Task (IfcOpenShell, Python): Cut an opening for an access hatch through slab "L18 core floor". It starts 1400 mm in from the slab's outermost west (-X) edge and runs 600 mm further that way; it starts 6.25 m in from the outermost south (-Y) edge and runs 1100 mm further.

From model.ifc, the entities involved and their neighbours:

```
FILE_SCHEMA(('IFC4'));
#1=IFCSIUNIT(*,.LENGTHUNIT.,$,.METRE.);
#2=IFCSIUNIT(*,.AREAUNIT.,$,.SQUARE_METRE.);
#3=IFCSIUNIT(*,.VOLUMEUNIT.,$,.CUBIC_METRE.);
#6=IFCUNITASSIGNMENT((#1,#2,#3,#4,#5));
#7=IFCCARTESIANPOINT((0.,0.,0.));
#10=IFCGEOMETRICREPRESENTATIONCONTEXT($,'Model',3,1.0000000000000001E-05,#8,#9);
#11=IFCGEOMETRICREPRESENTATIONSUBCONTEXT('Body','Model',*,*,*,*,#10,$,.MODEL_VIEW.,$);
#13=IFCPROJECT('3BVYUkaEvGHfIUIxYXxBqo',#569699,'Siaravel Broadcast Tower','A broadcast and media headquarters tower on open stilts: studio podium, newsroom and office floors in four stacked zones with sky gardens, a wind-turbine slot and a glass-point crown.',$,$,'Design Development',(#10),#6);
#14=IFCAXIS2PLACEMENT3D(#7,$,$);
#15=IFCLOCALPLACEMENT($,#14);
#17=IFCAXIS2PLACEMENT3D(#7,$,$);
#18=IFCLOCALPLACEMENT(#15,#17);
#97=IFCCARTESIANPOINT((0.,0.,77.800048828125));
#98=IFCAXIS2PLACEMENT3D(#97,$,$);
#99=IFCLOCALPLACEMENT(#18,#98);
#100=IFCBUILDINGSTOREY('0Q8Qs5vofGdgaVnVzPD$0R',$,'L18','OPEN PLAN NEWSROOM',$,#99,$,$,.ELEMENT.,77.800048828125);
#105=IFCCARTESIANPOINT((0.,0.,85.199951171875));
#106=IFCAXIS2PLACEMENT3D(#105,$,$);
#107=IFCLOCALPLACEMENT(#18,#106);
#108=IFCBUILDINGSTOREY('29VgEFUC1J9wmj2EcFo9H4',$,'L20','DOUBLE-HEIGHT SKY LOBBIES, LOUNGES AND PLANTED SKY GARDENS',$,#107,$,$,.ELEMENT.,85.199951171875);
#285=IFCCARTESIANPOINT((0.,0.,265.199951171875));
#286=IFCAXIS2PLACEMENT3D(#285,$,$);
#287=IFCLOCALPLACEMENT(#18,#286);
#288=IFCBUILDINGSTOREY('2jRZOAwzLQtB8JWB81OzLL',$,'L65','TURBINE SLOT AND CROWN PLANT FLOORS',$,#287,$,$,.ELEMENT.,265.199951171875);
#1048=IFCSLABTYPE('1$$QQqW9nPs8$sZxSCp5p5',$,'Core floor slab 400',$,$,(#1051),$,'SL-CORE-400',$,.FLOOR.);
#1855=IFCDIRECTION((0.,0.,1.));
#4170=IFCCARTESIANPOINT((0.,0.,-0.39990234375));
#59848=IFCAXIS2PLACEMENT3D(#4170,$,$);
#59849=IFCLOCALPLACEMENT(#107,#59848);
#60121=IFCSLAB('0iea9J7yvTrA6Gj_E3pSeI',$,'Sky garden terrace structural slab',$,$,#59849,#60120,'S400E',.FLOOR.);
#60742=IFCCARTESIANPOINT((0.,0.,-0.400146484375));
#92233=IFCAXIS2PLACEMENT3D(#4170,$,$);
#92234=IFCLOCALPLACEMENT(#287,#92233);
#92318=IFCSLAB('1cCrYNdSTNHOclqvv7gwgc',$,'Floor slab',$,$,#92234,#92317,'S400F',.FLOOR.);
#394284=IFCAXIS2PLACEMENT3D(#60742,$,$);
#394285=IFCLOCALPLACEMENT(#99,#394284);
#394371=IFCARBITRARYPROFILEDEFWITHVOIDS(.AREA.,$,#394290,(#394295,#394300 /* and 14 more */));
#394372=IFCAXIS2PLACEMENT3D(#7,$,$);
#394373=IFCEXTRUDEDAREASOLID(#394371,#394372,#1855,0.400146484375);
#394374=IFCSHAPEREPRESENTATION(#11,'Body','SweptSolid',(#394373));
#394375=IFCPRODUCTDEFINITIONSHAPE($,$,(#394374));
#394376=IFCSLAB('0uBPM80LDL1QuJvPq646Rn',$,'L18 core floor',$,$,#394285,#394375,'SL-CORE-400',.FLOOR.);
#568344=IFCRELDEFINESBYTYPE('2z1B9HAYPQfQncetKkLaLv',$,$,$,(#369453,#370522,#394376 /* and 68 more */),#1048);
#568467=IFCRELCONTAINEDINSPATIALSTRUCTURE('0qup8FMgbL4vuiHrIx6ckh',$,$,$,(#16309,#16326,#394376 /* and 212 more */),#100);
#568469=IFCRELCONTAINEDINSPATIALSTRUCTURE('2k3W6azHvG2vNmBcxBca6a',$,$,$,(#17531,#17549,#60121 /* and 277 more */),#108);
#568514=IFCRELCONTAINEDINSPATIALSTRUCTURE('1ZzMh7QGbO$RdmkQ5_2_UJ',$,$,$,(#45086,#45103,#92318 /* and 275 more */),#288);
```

```python
import numpy as np
import ifcopenshell
import ifcopenshell.api.feature
import ifcopenshell.api.geometry
import ifcopenshell.api.root
import ifcopenshell.geom
import ifcopenshell.util.placement
import ifcopenshell.util.representation
import ifcopenshell.util.shape
import ifcopenshell.util.unit

model = ifcopenshell.open("model.ifc")
unit_scale = ifcopenshell.util.unit.calculate_unit_scale(model)
settings = ifcopenshell.geom.settings()


def volume(element):
    """Net volume in cubic metres, openings subtracted."""
    shape = ifcopenshell.geom.create_shape(settings, element)
    return ifcopenshell.util.shape.get_volume(shape.geometry)


slab = model.by_guid("0uBPM80LDL1QuJvPq646Rn")
before = volume(slab)

# Extent in the slab's own axes, in metres. The edges named are its -X and -Y sides.
slab_shape = ifcopenshell.geom.create_shape(settings, slab)
vertices = ifcopenshell.util.shape.get_vertices(slab_shape.geometry)
x_min, y_min, bottom = vertices.min(axis=0)
top = vertices[:, 2].max()

opening = ifcopenshell.api.root.create_entity(model, ifc_class="IfcOpeningElement", name="Access hatch opening", predefined_type="OPENING")
context = ifcopenshell.util.representation.get_context(model, "Model", "Body", "MODEL_VIEW")
width, depth = 0.6, 1.1
outline = [(0.0, 0.0), (width, 0.0), (width, depth), (0.0, depth), (0.0, 0.0)]
# Overshoot both faces by 50 mm so the cut is clean.
shape = ifcopenshell.api.geometry.add_slab_representation(
    model, context=context, depth=top - bottom + 0.1, polyline=outline
)
ifcopenshell.api.geometry.assign_representation(model, product=opening, representation=shape)

matrix = ifcopenshell.util.placement.get_local_placement(slab.ObjectPlacement)
matrix[:, 3] = matrix @ np.append(np.array([x_min + 1.4, y_min + 6.25, bottom - 0.05]) / unit_scale, 1.0)
ifcopenshell.api.geometry.edit_object_placement(model, product=opening, matrix=matrix, is_si=False)
ifcopenshell.api.feature.add_feature(model, feature=opening, element=slab)

after = volume(slab)

print(f"slab volume {before:.3f} -> {after:.3f} m3")

model.write("model_updated.ifc")
```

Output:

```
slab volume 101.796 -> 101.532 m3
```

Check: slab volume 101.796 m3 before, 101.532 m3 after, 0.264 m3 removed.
